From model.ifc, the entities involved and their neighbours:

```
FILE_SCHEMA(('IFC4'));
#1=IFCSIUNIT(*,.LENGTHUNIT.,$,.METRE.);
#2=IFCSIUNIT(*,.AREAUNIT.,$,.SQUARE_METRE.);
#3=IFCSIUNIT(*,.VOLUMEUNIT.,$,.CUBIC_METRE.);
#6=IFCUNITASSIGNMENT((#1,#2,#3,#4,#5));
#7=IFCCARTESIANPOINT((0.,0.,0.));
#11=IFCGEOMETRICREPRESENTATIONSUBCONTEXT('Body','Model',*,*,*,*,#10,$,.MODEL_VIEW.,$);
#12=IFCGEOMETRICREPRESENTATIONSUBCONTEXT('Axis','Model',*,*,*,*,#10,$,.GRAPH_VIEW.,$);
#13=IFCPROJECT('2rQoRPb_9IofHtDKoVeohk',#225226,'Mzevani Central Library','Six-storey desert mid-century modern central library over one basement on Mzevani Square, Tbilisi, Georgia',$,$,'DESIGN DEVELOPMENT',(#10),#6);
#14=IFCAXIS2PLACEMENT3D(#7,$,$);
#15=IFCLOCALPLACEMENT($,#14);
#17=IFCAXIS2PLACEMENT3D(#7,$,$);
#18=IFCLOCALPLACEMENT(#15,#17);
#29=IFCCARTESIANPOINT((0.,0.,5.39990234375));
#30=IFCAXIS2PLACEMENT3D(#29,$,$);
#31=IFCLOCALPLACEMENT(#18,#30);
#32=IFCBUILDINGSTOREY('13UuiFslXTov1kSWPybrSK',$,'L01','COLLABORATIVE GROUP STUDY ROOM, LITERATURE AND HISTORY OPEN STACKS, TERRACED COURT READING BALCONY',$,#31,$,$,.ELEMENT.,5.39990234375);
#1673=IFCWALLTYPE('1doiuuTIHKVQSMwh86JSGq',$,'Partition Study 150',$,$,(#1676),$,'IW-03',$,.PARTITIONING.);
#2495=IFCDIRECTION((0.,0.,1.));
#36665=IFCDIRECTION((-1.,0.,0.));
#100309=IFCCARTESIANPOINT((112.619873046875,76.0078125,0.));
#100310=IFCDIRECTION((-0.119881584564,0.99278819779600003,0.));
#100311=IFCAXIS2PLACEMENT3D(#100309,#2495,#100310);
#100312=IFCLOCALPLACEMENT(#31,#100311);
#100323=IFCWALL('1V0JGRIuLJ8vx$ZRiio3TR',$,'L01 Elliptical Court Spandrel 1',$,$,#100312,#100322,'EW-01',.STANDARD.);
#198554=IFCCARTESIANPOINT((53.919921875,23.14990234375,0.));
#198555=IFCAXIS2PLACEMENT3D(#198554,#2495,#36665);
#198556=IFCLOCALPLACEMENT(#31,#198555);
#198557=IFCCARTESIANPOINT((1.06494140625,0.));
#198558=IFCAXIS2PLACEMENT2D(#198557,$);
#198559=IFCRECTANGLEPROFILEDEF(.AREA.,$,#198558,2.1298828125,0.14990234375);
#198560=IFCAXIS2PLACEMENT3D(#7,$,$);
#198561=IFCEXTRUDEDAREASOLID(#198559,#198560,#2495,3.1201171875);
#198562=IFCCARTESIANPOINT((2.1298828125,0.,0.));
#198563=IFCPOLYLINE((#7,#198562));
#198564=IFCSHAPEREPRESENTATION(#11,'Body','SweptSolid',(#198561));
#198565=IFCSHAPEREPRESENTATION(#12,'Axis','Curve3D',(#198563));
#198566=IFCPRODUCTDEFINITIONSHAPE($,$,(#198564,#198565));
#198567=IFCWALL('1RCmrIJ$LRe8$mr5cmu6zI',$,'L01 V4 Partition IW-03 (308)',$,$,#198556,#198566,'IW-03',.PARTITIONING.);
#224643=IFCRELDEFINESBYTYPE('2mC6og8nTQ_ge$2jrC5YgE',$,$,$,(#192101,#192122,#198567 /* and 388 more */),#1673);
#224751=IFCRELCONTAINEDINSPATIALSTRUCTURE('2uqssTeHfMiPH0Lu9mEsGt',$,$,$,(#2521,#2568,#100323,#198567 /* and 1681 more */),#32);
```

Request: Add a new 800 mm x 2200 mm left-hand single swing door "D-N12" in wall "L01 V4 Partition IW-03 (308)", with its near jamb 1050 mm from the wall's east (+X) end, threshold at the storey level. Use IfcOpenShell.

```python
import numpy as np
import ifcopenshell
import ifcopenshell.api.feature
import ifcopenshell.api.geometry
import ifcopenshell.api.root
import ifcopenshell.api.spatial
import ifcopenshell.geom
import ifcopenshell.util.element
import ifcopenshell.util.placement
import ifcopenshell.util.representation
import ifcopenshell.util.shape
import ifcopenshell.util.unit

model = ifcopenshell.open("model.ifc")
unit_scale = ifcopenshell.util.unit.calculate_unit_scale(model)
settings = ifcopenshell.geom.settings()


def volume(element):
    """Net volume in cubic metres, openings subtracted."""
    shape = ifcopenshell.geom.create_shape(settings, element)
    return ifcopenshell.util.shape.get_volume(shape.geometry)


wall = model.by_guid("1RCmrIJ$LRe8$mr5cmu6zI")
storey = ifcopenshell.util.element.get_container(wall, ifc_class="IfcBuildingStorey")
context = ifcopenshell.util.representation.get_context(model, "Model", "Body", "MODEL_VIEW")
before = volume(wall)

width, height, from_end, sill = 0.8, 2.2, 1.05, 0.0  # metres

# The wall runs along its own X axis, and the end named is its -X end.
wall_shape = ifcopenshell.geom.create_shape(settings, wall)
x, y, z = ifcopenshell.util.shape.get_vertices(wall_shape.geometry).T
start = x.min() + from_end
face, thickness = float(y.min()), float(y.max() - y.min())
wall_matrix = ifcopenshell.util.placement.get_local_placement(wall.ObjectPlacement)
level = ifcopenshell.util.placement.get_local_placement(storey.ObjectPlacement)[2, 3]


def in_wall(x, y):
    """Placement at x, y metres in the wall's axes, at sill height."""
    matrix = wall_matrix.copy()
    matrix[:, 3] = wall_matrix @ np.array([x / unit_scale, y / unit_scale, 0.0, 1.0])
    matrix[2, 3] = level + sill / unit_scale
    return matrix


# Opening: a box that overshoots both wall faces by 50 mm.
opening = ifcopenshell.api.root.create_entity(model, ifc_class="IfcOpeningElement", predefined_type="OPENING")
box = ifcopenshell.api.geometry.add_wall_representation(
    model, context=context, length=width, height=height, thickness=thickness + 0.1
)
ifcopenshell.api.geometry.assign_representation(model, product=opening, representation=box)
ifcopenshell.api.geometry.edit_object_placement(model, product=opening, matrix=in_wall(start, face - 0.05), is_si=False)
ifcopenshell.api.feature.add_feature(model, feature=opening, element=wall)

door = ifcopenshell.api.root.create_entity(model, ifc_class="IfcDoor", name="D-N12", predefined_type="DOOR")
door.OverallWidth, door.OverallHeight = width / unit_scale, height / unit_scale
door.OperationType = "SINGLE_SWING_LEFT"
body = ifcopenshell.api.geometry.add_door_representation(
    model,
    context=context,
    overall_width=door.OverallWidth,
    overall_height=door.OverallHeight,
    operation_type="SINGLE_SWING_LEFT",
    lining_properties={"LiningDepth": thickness / unit_scale, "ThresholdDepth": thickness / unit_scale},
)
ifcopenshell.api.geometry.assign_representation(model, product=door, representation=body)
ifcopenshell.api.spatial.assign_container(model, products=[door], relating_structure=storey)
ifcopenshell.api.feature.add_filling(model, opening=opening, element=door)

# The lining spans the wall, so the door starts at the wall face.
ifcopenshell.api.geometry.edit_object_placement(model, product=door, matrix=in_wall(start, face), is_si=False)

after = volume(wall)

print(f"wall volume {before:.3f} -> {after:.3f} m3")

model.write("model_updated.ifc")
```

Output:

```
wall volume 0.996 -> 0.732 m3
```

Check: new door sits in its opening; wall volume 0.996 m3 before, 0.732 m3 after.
